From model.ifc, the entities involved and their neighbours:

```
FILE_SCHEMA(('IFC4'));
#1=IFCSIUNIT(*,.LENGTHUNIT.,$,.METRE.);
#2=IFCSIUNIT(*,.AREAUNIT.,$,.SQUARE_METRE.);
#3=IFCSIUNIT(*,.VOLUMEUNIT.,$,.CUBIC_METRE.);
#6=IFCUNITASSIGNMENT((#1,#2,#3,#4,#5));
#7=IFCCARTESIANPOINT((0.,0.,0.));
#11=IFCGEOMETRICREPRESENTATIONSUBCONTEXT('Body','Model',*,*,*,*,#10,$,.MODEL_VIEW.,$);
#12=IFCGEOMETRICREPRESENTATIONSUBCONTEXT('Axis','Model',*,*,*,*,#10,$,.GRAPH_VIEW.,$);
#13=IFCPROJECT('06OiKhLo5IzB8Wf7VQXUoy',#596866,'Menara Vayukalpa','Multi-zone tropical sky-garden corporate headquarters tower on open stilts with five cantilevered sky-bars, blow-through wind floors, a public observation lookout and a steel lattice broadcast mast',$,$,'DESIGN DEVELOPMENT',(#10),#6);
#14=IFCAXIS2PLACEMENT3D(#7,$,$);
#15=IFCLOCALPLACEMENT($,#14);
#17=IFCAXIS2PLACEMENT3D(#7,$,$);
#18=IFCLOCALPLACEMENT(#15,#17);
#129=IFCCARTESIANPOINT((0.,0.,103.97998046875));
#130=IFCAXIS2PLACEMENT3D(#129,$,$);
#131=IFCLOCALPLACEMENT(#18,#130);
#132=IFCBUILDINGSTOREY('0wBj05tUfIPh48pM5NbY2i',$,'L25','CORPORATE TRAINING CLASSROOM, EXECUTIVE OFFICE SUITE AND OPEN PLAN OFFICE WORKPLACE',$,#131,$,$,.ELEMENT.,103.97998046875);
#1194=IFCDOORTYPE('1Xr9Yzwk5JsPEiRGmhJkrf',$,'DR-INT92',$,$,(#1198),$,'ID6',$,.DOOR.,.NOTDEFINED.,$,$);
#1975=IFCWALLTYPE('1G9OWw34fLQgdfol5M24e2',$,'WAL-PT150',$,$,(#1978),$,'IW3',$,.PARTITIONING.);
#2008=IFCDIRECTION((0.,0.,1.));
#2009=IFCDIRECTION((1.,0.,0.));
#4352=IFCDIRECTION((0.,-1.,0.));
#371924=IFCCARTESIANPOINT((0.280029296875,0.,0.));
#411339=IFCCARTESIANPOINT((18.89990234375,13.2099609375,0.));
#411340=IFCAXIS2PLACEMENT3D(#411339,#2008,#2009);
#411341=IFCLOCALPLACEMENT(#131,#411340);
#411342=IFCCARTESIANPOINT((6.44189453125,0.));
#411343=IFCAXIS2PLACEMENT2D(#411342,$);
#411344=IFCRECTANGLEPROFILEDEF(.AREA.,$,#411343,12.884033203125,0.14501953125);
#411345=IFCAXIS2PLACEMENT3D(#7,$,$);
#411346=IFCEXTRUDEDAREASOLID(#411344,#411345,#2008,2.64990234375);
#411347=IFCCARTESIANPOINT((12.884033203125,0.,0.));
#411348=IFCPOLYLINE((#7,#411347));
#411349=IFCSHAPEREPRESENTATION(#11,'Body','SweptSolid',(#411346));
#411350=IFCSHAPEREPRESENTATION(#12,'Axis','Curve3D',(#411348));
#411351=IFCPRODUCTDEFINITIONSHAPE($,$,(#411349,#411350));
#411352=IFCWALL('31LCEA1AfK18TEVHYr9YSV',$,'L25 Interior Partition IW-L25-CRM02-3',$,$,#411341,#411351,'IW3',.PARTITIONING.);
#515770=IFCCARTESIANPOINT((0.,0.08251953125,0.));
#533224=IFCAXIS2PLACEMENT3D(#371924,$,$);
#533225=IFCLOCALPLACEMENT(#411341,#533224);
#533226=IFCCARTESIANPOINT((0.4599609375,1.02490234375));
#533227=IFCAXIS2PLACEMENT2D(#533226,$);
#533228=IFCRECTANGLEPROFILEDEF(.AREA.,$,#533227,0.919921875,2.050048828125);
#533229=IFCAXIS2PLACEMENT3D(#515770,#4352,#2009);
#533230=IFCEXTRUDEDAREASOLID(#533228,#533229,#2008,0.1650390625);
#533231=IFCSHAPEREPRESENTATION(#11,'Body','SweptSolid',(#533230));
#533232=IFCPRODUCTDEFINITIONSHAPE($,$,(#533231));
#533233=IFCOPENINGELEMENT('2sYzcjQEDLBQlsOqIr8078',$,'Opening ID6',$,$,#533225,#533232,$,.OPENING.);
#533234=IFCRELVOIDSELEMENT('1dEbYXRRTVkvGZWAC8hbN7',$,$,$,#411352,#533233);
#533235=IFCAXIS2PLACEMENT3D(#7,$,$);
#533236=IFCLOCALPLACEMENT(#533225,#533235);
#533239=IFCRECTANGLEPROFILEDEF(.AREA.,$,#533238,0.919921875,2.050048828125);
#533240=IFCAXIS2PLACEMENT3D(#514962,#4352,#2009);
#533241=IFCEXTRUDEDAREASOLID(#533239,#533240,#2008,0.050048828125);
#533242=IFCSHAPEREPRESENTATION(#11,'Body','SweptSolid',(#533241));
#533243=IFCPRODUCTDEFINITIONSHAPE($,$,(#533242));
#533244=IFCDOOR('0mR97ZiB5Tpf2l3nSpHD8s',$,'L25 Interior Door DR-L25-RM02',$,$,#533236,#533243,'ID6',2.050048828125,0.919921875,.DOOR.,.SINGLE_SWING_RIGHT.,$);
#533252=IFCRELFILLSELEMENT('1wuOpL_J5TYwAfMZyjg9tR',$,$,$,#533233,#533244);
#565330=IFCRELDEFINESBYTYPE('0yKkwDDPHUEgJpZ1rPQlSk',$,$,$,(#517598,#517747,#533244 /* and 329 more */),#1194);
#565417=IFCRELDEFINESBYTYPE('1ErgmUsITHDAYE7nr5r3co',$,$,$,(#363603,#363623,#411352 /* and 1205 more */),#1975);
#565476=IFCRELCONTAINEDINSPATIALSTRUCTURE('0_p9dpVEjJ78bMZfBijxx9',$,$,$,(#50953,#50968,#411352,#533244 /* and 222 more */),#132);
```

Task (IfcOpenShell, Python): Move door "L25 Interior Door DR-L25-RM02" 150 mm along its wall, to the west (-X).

```python
import ifcopenshell
import ifcopenshell.api.geometry
import ifcopenshell.util.placement
import ifcopenshell.util.unit

model = ifcopenshell.open("model.ifc")
unit_scale = ifcopenshell.util.unit.calculate_unit_scale(model)

door = model.by_guid("0mR97ZiB5Tpf2l3nSpHD8s")
opening = door.FillsVoids[0].RelatingOpeningElement
wall = opening.VoidsElements[0].RelatingBuildingElement

wall_matrix = ifcopenshell.util.placement.get_local_placement(wall.ObjectPlacement)
shift = wall_matrix[:3, 0] * -0.15 / unit_scale
before = ifcopenshell.util.placement.get_local_placement(door.ObjectPlacement)[:3, 3].copy()

# The door is placed relative to its opening, so it follows when the opening moves.
matrix = ifcopenshell.util.placement.get_local_placement(opening.ObjectPlacement)
matrix[:3, 3] += shift
ifcopenshell.api.geometry.edit_object_placement(
    model, product=opening, matrix=matrix, is_si=False, should_transform_children=True
)

after = ifcopenshell.util.placement.get_local_placement(door.ObjectPlacement)[:3, 3]
print("door moved by", (after - before).round(3) + 0.0)

model.write("model_rev.ifc")
```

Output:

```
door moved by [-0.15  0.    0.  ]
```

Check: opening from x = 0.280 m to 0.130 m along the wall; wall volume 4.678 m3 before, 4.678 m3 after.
